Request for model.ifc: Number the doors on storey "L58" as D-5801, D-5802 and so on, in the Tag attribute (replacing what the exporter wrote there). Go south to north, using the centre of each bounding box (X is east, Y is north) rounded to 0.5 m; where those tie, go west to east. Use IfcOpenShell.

First a look at what the model holds.

```python
import ifcopenshell
import ifcopenshell.util.element
import ifcopenshell.util.placement

model = ifcopenshell.open("model.ifc")
print(model.schema)
storey = next(s for s in model.by_type("IfcBuildingStorey") if s.Name == "L58")
doors = [e for e in ifcopenshell.util.element.get_decomposition(storey) if e.is_a("IfcDoor")]
for e in sorted(doors, key=lambda e: e.id()):
    origin = ifcopenshell.util.placement.get_local_placement(e.ObjectPlacement)[:3, 3]
    print(e.id(), e.Tag, e.Name, origin.round(2) + 0.0, sep=" | ")
```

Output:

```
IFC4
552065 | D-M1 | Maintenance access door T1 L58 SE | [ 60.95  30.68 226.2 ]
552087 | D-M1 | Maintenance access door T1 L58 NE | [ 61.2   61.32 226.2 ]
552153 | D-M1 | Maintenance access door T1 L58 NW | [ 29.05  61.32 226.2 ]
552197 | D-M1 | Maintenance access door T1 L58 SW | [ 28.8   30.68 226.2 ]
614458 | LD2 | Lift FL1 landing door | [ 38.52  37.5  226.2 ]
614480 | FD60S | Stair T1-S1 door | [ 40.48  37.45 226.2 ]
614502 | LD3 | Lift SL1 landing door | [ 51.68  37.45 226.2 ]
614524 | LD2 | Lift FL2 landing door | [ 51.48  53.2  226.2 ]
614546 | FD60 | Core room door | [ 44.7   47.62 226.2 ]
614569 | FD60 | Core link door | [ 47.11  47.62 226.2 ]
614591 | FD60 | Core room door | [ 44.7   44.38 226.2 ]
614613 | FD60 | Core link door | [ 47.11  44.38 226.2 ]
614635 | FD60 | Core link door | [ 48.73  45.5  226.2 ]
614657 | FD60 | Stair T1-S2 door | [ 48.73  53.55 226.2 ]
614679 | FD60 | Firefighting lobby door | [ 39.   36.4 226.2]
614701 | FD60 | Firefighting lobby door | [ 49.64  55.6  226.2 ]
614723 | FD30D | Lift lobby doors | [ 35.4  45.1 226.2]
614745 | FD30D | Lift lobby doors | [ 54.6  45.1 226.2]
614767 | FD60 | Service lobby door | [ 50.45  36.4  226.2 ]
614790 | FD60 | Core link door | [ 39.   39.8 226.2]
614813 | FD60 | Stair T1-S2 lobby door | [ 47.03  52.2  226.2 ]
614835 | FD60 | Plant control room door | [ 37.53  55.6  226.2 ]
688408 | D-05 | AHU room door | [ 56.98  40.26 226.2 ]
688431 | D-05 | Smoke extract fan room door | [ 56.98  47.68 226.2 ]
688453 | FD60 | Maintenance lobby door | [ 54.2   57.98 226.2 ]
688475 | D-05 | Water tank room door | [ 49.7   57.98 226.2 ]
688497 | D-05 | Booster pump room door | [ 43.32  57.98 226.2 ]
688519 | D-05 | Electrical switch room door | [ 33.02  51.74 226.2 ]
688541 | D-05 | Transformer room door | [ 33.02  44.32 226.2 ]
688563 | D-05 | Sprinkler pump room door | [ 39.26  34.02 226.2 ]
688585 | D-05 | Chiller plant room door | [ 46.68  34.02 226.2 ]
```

```python
import ifcopenshell
import ifcopenshell.geom
import ifcopenshell.util.element
import ifcopenshell.util.shape

model = ifcopenshell.open("model.ifc")
settings = ifcopenshell.geom.settings()
settings.set("use-world-coords", True)


def centre(element):
    shape = ifcopenshell.geom.create_shape(settings, element)
    return ifcopenshell.util.shape.get_bbox_centroid(shape.geometry)


storey = next(s for s in model.by_type("IfcBuildingStorey") if s.Name == "L58")
doors = [e for e in ifcopenshell.util.element.get_decomposition(storey) if e.is_a("IfcDoor")]

# Insertion points can sit at a corner or the storey origin, so sort by the geometry (in metres).
centres = {e: centre(e) for e in doors}
doors.sort(key=lambda e: (round(centres[e][1] / 0.5), centres[e][0]))

for i, e in enumerate(doors, start=1):
    number = f"D-58{i:02d}"
    e.Tag = number
    print(e.id(), number)

model.write("model_updated.ifc")
```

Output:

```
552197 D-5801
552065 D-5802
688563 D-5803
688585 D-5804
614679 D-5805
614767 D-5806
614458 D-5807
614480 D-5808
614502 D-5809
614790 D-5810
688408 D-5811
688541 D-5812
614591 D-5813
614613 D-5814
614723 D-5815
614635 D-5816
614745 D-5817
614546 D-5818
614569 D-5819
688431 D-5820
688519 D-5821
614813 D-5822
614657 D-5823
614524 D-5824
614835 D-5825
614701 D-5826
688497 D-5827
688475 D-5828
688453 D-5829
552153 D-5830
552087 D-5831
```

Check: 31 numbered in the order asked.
